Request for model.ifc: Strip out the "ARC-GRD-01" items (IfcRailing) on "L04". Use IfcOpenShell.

First a look at what the model holds.

```python
import ifcopenshell
import ifcopenshell.util.element

model = ifcopenshell.open("model.ifc")
print(model.schema)
storey = next(s for s in model.by_type("IfcBuildingStorey") if s.Name == "L04")
railings = [e for e in ifcopenshell.util.element.get_decomposition(storey) if e.is_a("IfcRailing")]
seen = {}
for e in railings:
    element_type = ifcopenshell.util.element.get_type(e)
    name = element_type.Name if element_type not in (None, e) else None
    seen[name] = seen.get(name, 0) + 1
for name, count in sorted(seen.items(), key=str):
    print(count, "x", name)
```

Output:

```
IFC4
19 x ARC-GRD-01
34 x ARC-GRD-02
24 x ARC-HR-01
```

```python
import ifcopenshell
import ifcopenshell.api.root
import ifcopenshell.util.element

model = ifcopenshell.open("model.ifc")

storey = next(s for s in model.by_type("IfcBuildingStorey") if s.Name == "L04")
railings = [e for e in ifcopenshell.util.element.get_decomposition(storey) if e.is_a("IfcRailing")]
targets = [e for e in railings if (t := ifcopenshell.util.element.get_type(e)) not in (None, e) and t.Name == "ARC-GRD-01"]

for e in targets:
    ifcopenshell.api.root.remove_product(model, product=e)
print(len(targets), "removed")

model.write("model-out.ifc")
```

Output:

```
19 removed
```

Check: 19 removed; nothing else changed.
